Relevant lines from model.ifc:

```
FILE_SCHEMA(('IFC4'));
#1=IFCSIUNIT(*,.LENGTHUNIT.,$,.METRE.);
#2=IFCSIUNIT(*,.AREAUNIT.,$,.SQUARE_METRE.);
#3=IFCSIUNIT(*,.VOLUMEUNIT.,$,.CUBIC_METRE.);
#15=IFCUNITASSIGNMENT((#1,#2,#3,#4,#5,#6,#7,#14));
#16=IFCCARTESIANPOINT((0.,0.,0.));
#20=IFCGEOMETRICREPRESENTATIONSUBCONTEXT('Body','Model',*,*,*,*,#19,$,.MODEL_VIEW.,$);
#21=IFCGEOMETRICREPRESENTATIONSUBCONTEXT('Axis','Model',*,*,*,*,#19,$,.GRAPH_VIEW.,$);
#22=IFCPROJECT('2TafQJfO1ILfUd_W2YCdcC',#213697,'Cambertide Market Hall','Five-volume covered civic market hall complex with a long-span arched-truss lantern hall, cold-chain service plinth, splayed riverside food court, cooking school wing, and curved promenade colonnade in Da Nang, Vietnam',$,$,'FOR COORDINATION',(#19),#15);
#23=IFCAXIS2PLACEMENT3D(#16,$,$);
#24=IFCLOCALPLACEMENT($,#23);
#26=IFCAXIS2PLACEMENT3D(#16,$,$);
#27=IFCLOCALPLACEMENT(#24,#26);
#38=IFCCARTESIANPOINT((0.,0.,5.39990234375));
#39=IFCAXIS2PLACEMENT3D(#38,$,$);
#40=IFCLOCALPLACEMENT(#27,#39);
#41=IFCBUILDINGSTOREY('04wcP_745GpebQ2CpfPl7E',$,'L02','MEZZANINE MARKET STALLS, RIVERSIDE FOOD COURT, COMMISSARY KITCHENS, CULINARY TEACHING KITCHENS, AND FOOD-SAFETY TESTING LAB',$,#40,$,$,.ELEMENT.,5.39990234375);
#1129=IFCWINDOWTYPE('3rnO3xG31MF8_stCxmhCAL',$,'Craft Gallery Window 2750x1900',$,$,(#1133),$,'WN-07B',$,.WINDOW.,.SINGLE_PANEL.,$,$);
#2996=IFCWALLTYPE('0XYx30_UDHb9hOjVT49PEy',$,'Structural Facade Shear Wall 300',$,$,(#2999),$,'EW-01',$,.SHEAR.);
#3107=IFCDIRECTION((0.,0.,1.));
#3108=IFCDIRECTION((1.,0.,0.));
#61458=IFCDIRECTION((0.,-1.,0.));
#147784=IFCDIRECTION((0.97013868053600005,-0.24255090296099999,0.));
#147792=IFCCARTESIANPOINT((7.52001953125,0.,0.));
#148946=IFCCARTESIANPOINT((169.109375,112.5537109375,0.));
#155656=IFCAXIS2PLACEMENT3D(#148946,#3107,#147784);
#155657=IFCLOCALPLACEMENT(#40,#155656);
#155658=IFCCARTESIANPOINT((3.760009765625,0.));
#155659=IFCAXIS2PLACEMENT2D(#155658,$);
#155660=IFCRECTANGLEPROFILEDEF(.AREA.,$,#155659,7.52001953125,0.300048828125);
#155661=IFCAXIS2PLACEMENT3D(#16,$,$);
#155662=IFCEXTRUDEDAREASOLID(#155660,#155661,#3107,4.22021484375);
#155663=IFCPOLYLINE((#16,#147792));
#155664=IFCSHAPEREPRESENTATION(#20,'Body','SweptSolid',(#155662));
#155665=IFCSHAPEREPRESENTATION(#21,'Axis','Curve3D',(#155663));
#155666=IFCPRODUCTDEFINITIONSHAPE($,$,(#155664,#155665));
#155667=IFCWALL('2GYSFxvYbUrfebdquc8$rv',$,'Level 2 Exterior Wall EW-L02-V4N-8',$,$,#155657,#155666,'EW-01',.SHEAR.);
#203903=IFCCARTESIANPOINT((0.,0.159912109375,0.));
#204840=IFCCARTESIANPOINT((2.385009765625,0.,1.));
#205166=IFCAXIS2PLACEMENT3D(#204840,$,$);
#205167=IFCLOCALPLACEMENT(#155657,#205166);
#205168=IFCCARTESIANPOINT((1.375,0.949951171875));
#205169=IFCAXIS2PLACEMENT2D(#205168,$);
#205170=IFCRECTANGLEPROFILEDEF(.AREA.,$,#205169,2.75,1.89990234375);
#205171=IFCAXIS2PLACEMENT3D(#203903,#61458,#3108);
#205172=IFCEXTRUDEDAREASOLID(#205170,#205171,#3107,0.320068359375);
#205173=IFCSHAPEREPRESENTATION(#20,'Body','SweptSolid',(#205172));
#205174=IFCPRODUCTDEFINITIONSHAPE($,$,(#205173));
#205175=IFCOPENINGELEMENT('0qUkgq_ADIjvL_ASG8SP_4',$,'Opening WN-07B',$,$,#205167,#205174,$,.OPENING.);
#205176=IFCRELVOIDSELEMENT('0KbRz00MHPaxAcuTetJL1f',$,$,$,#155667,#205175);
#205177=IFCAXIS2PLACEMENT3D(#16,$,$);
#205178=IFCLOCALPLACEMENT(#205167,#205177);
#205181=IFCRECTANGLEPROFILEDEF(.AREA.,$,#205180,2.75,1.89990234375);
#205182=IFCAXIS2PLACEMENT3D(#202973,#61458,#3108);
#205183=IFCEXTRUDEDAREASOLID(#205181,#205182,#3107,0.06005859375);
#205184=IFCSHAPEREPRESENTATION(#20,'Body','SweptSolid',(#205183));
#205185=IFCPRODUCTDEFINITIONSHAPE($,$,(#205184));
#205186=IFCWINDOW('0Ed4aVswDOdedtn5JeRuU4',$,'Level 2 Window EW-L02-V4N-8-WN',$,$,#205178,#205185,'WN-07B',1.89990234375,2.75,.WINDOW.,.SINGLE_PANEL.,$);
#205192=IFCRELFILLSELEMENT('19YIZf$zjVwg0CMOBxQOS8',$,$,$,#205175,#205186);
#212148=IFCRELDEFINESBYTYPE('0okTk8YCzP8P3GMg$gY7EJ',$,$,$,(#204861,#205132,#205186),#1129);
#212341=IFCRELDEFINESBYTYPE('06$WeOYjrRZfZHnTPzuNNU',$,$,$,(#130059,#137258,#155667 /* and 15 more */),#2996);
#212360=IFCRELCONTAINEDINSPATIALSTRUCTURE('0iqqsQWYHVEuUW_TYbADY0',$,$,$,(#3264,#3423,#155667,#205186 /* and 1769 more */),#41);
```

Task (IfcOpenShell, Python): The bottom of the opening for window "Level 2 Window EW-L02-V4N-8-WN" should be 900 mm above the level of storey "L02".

```python
import numpy as np
import ifcopenshell
import ifcopenshell.api.geometry
import ifcopenshell.geom
import ifcopenshell.util.element
import ifcopenshell.util.placement
import ifcopenshell.util.shape
import ifcopenshell.util.unit

model = ifcopenshell.open("model.ifc")
unit_scale = ifcopenshell.util.unit.calculate_unit_scale(model)

window = model.by_id(205186)
opening = window.FillsVoids[0].RelatingOpeningElement
storey = ifcopenshell.util.element.get_container(window, ifc_class="IfcBuildingStorey")
level = ifcopenshell.util.placement.get_local_placement(storey.ObjectPlacement)[2, 3]

# The opening's origin need not be at the sill, so measure its lowest point.
shape = ifcopenshell.geom.create_shape(ifcopenshell.geom.settings(), opening)
bottom = ifcopenshell.util.shape.get_shape_bottom_elevation(shape, shape.geometry) / unit_scale
dz = level + 0.9 / unit_scale - bottom

shift = np.array([0.0, 0.0, dz])
# The window is placed relative to its opening, so it follows when the opening moves.
matrix = ifcopenshell.util.placement.get_local_placement(opening.ObjectPlacement)
matrix[:3, 3] += shift
ifcopenshell.api.geometry.edit_object_placement(
    model, product=opening, matrix=matrix, is_si=False, should_transform_children=True
)

print(f"moved by {dz * unit_scale:+.3f} m")

model.write("model_edited.ifc")
```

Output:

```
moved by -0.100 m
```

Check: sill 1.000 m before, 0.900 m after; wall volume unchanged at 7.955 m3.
